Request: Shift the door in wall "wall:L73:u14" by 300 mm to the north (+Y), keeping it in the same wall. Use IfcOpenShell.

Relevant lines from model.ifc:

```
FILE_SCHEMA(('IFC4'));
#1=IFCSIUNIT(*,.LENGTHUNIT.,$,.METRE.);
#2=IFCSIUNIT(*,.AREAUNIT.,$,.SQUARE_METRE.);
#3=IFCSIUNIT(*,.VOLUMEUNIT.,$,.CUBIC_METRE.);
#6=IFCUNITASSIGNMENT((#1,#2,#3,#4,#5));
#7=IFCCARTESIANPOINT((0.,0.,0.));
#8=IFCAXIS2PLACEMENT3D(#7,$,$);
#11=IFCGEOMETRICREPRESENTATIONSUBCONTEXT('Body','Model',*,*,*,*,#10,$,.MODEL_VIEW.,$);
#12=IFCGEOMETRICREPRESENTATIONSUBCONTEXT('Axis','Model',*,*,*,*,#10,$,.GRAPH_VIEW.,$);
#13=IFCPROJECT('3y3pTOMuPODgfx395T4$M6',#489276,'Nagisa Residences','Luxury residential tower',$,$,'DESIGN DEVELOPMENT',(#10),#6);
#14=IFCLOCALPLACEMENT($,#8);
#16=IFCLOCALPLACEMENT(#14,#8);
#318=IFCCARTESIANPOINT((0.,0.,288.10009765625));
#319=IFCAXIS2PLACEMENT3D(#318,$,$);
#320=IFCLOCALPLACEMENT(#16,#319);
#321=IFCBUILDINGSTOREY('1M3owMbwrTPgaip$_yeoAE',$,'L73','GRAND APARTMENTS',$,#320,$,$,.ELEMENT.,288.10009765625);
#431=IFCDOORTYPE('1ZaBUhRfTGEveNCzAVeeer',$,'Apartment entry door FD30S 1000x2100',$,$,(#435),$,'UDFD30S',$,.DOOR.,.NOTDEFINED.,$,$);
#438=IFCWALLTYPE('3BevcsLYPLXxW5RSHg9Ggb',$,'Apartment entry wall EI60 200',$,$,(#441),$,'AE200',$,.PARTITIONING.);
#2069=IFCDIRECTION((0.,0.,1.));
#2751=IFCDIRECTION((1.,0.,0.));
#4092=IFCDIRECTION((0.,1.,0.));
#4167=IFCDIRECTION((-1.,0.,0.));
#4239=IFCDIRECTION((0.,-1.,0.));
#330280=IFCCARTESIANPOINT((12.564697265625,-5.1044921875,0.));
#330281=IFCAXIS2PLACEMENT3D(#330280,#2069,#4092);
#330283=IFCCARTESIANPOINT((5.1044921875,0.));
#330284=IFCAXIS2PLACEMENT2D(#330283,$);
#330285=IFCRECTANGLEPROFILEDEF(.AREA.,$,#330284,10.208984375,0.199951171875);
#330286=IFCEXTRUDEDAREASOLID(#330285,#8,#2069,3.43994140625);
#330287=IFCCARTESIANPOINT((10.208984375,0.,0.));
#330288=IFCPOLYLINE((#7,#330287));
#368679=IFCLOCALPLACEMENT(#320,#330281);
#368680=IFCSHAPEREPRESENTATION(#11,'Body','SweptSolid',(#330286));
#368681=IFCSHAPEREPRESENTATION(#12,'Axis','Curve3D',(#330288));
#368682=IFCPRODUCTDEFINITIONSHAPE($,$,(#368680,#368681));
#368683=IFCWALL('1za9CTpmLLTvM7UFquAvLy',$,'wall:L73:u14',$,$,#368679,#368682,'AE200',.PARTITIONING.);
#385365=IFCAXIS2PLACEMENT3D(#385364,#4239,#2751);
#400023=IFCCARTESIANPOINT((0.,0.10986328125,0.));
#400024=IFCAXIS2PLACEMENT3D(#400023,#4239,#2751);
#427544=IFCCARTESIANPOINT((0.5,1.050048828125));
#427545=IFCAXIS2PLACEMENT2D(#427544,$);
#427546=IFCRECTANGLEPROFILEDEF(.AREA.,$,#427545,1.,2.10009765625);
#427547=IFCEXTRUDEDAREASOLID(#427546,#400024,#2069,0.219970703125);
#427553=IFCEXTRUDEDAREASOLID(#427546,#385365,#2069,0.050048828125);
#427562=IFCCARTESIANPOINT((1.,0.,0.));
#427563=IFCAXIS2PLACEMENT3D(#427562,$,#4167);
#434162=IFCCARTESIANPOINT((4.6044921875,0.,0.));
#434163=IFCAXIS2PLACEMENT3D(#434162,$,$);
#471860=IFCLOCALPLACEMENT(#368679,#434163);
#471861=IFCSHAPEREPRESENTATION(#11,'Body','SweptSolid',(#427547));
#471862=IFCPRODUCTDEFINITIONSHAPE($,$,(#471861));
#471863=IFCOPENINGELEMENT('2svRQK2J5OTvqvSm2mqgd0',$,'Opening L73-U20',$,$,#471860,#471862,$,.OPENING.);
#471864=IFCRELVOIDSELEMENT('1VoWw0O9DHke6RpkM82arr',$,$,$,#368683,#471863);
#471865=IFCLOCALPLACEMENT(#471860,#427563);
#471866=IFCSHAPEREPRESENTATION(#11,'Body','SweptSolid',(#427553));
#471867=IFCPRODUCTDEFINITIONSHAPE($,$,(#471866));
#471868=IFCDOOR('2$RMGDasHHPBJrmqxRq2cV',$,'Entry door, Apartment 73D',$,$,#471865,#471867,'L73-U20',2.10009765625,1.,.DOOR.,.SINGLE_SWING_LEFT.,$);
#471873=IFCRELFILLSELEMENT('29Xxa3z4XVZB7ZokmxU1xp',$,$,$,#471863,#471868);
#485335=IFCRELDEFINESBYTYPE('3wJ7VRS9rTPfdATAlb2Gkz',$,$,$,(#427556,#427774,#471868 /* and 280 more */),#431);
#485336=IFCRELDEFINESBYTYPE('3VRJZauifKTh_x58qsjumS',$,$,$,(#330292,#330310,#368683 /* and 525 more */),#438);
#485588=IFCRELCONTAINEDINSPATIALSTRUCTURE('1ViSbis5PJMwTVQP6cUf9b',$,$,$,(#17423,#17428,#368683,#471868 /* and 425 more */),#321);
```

```python
import ifcopenshell
import ifcopenshell.api.geometry
import ifcopenshell.util.placement

model = ifcopenshell.open("model.ifc")

door = model.by_guid("2$RMGDasHHPBJrmqxRq2cV")
opening = door.FillsVoids[0].RelatingOpeningElement
wall = opening.VoidsElements[0].RelatingBuildingElement

wall_matrix = ifcopenshell.util.placement.get_local_placement(wall.ObjectPlacement)
shift = wall_matrix[:3, 0] * 0.3
before = ifcopenshell.util.placement.get_local_placement(door.ObjectPlacement)[:3, 3].copy()

# The door is placed relative to its opening, so it follows when the opening moves.
matrix = ifcopenshell.util.placement.get_local_placement(opening.ObjectPlacement)
matrix[:3, 3] += shift
ifcopenshell.api.geometry.edit_object_placement(
    model, product=opening, matrix=matrix, is_si=False, should_transform_children=True
)

after = ifcopenshell.util.placement.get_local_placement(door.ObjectPlacement)[:3, 3]
print("door moved by", (after - before).round(3) + 0.0)

model.write("model_v2.ifc")
```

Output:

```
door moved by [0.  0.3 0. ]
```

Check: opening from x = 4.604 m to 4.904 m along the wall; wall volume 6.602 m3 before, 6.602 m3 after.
